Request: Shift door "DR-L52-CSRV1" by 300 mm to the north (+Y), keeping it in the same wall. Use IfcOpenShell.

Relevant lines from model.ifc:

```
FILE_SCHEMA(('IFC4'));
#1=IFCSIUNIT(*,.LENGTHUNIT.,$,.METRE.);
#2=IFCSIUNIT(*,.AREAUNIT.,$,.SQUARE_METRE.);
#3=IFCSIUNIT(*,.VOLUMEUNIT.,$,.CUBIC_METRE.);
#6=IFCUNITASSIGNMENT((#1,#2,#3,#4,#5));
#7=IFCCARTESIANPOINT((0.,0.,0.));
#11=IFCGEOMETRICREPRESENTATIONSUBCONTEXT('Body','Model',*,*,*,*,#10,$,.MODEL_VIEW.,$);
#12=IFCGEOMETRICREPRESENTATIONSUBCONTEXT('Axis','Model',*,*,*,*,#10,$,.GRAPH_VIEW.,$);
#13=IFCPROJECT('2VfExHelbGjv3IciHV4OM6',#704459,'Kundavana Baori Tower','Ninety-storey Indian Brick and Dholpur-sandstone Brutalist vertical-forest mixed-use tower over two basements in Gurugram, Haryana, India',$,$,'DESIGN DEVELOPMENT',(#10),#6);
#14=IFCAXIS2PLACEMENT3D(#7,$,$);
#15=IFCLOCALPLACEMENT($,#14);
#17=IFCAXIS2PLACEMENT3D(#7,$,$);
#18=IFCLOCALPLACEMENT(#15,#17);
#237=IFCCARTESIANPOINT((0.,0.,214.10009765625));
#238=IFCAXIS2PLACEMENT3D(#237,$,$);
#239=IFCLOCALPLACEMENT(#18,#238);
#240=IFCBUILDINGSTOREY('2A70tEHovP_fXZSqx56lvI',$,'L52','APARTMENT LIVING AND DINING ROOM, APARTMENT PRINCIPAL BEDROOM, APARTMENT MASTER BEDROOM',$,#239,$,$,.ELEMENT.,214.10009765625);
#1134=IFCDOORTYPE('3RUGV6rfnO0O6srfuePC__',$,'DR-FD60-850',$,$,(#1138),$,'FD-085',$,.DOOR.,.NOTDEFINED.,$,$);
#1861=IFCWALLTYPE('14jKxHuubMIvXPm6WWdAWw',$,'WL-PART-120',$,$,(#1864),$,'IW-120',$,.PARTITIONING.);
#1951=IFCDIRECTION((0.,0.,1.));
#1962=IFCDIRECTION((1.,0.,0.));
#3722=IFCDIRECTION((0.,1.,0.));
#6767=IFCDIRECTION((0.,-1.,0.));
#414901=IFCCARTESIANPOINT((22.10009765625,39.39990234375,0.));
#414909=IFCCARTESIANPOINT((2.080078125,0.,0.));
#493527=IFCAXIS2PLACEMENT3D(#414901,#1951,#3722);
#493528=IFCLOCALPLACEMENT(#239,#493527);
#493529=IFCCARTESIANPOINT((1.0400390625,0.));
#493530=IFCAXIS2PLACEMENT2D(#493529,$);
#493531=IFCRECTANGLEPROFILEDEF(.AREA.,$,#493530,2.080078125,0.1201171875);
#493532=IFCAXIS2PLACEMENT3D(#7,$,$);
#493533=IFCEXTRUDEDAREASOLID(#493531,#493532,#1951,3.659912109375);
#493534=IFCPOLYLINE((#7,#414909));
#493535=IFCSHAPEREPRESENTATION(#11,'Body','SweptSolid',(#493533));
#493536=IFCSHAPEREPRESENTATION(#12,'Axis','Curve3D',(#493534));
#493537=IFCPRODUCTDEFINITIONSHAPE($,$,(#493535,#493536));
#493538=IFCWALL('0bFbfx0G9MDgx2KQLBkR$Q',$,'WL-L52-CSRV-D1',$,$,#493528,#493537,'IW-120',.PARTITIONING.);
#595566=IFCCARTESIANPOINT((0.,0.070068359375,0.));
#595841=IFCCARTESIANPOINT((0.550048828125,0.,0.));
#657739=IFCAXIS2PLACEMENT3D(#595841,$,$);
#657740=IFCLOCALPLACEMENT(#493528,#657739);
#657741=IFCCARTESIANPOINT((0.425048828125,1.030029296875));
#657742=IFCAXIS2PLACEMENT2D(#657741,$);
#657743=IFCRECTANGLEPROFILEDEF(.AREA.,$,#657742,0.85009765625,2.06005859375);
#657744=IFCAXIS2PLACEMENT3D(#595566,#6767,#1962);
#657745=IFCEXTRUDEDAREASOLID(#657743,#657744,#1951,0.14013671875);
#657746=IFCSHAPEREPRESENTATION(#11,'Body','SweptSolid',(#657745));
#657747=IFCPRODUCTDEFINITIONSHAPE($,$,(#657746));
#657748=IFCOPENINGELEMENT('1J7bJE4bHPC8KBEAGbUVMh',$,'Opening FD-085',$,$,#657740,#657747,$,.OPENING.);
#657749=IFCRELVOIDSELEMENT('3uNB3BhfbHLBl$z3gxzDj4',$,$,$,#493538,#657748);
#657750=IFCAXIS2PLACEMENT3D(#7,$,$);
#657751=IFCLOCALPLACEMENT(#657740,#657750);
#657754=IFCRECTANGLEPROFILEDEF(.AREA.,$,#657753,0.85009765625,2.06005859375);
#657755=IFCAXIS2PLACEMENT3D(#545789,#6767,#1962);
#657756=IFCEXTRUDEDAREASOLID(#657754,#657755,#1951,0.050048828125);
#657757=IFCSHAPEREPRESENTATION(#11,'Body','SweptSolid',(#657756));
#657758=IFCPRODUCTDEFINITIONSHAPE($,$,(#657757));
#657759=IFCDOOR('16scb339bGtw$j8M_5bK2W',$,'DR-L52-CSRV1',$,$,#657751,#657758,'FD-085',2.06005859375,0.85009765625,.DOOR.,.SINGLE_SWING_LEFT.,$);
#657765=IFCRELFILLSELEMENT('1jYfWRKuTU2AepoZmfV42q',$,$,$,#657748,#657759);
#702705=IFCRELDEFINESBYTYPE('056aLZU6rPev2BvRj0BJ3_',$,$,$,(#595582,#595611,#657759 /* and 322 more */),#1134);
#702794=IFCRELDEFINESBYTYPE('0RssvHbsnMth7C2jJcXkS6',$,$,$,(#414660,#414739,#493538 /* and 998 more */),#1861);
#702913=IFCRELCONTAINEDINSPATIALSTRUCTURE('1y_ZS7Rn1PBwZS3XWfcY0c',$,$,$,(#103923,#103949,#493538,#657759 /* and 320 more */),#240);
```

```python
import ifcopenshell
import ifcopenshell.api.geometry
import ifcopenshell.util.placement
import ifcopenshell.util.unit

model = ifcopenshell.open("model.ifc")
unit_scale = ifcopenshell.util.unit.calculate_unit_scale(model)

door = model.by_id(657759)
opening = door.FillsVoids[0].RelatingOpeningElement
wall = opening.VoidsElements[0].RelatingBuildingElement

wall_matrix = ifcopenshell.util.placement.get_local_placement(wall.ObjectPlacement)
shift = wall_matrix[:3, 0] * 0.3 / unit_scale
before = ifcopenshell.util.placement.get_local_placement(door.ObjectPlacement)[:3, 3].copy()

# The door is placed relative to its opening, so it follows when the opening moves.
matrix = ifcopenshell.util.placement.get_local_placement(opening.ObjectPlacement)
matrix[:3, 3] += shift
ifcopenshell.api.geometry.edit_object_placement(
    model, product=opening, matrix=matrix, is_si=False, should_transform_children=True
)

after = ifcopenshell.util.placement.get_local_placement(door.ObjectPlacement)[:3, 3]
print("door moved by", (after - before).round(3) + 0.0)

model.write("model-out.ifc")
```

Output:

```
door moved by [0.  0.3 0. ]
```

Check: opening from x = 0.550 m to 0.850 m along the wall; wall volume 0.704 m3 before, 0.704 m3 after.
